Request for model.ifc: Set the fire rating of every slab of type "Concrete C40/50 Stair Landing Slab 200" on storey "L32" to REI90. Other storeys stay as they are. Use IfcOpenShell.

First a look at what the model holds.

```python
import ifcopenshell
import ifcopenshell.util.element

model = ifcopenshell.open("model.ifc")
print(model.schema)
storey = next(s for s in model.by_type("IfcBuildingStorey") if s.Name == "L32")
slabs = [e for e in ifcopenshell.util.element.get_decomposition(storey) if e.is_a("IfcSlab")]
seen = {}
for e in slabs:
    element_type = ifcopenshell.util.element.get_type(e)
    key = (element_type.Name if element_type != e and element_type else None, ifcopenshell.util.element.get_pset(e, "Pset_SlabCommon", "FireRating"))
    seen[key] = seen.get(key, 0) + 1
for (name, value), count in sorted(seen.items(), key=str):
    print(count, "x", name, "|", value)
```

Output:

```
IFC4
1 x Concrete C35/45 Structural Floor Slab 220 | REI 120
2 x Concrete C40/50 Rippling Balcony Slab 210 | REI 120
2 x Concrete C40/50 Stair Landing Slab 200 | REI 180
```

```python
import ifcopenshell
import ifcopenshell.api.pset
import ifcopenshell.util.element

model = ifcopenshell.open("model.ifc")

storey = next(s for s in model.by_type("IfcBuildingStorey") if s.Name == "L32")
slabs = [e for e in ifcopenshell.util.element.get_decomposition(storey) if e.is_a("IfcSlab")]

count = 0
for e in slabs:
    element_type = ifcopenshell.util.element.get_type(e)
    if element_type in (None, e) or element_type.Name != "Concrete C40/50 Stair Landing Slab 200":
        continue
    found = ifcopenshell.util.element.get_pset(e, "Pset_SlabCommon", should_inherit=False)
    if found:
        pset = model.by_id(found["id"])
        if len(ifcopenshell.util.element.get_elements_by_pset(pset)) > 1:
            pset = ifcopenshell.api.pset.unshare_pset(model, products=[e], pset=pset)[0]
    else:
        pset = ifcopenshell.api.pset.add_pset(model, product=e, name="Pset_SlabCommon")
    ifcopenshell.api.pset.edit_pset(model, pset=pset, properties={"FireRating": "REI90"})
    count += 1

print(count, "slabs updated")

model.write("model-out.ifc")
```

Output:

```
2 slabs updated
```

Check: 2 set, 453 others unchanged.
